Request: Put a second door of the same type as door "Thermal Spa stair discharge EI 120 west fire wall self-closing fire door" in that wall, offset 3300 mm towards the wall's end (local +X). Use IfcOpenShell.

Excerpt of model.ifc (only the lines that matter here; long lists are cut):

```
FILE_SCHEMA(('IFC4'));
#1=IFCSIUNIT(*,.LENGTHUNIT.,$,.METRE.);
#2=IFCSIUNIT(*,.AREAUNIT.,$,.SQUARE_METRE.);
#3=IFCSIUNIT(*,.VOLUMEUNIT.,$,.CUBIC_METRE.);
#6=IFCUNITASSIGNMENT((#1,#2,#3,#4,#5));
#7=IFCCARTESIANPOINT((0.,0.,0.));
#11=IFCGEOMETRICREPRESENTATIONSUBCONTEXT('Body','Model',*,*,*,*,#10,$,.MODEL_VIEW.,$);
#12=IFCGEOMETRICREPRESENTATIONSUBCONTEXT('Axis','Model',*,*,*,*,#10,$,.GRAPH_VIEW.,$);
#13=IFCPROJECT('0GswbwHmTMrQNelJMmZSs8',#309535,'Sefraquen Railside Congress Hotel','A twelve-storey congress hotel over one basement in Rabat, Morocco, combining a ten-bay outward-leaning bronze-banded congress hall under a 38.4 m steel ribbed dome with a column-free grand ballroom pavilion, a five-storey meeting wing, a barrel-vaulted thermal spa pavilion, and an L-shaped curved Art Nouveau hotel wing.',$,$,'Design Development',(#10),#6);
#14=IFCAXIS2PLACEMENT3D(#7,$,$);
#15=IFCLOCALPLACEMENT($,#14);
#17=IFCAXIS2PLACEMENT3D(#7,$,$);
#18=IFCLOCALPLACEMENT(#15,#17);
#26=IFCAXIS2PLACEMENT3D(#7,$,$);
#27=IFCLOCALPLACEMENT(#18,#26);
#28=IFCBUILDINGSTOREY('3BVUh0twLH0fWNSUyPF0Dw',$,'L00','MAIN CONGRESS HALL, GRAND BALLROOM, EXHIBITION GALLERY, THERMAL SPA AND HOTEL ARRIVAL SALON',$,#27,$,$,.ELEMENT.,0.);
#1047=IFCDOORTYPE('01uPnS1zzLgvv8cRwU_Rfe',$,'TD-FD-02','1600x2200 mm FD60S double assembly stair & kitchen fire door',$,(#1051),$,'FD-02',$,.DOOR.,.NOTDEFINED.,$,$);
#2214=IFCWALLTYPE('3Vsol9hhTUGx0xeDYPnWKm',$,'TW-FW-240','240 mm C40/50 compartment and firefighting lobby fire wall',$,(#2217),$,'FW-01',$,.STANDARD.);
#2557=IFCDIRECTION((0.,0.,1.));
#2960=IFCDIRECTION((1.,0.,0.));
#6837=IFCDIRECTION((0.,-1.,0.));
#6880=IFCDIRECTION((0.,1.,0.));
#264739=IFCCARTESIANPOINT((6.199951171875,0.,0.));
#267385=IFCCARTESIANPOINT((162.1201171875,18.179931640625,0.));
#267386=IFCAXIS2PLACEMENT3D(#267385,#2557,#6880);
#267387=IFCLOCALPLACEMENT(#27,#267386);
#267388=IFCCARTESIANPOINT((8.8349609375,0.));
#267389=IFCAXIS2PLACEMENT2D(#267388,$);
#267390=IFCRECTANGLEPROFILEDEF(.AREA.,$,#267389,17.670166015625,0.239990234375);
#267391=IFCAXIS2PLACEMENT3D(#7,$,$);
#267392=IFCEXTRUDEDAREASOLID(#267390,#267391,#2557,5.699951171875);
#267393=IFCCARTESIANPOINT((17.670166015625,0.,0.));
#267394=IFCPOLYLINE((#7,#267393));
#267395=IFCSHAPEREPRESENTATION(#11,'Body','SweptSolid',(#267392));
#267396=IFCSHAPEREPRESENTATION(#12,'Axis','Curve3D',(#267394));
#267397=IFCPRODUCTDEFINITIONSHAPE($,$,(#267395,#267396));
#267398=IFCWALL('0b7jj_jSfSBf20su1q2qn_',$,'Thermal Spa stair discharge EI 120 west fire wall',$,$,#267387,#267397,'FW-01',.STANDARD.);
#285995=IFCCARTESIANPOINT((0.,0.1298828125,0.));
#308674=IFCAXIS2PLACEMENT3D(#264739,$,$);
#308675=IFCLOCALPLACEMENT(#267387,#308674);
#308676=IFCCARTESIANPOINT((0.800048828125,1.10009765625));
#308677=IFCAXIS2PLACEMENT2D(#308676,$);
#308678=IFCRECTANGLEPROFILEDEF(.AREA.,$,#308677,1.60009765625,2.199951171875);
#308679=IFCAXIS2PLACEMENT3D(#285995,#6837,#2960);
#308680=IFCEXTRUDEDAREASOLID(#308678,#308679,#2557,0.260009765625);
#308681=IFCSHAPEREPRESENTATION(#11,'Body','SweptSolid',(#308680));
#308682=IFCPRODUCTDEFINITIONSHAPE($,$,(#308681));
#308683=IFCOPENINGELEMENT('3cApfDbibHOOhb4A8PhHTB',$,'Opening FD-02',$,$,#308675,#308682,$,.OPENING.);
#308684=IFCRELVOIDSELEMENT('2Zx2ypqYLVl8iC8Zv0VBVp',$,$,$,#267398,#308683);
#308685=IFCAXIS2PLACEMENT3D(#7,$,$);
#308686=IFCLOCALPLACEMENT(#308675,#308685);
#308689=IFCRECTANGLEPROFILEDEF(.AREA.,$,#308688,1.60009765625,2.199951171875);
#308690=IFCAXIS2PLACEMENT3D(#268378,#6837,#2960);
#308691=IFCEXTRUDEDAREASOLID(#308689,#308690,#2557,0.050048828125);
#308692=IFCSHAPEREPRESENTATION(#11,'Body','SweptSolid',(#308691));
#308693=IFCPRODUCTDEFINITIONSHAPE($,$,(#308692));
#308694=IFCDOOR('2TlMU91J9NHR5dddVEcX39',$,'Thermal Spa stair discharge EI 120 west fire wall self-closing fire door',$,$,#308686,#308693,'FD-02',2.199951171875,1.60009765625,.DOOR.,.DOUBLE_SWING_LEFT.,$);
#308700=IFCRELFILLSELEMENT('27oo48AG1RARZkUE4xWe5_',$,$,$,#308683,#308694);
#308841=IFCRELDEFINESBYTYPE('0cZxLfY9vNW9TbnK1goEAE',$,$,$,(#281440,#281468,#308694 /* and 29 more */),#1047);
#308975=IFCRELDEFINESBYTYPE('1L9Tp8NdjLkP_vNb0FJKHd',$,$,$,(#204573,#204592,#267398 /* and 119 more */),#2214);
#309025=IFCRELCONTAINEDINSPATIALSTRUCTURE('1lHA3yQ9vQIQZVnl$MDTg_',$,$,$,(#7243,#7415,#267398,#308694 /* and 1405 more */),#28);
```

```python
import ifcopenshell
import ifcopenshell.api.feature
import ifcopenshell.api.geometry
import ifcopenshell.api.root
import ifcopenshell.geom
import ifcopenshell.util.element
import ifcopenshell.util.placement
import ifcopenshell.util.shape
import ifcopenshell.util.unit

model = ifcopenshell.open("model.ifc")
unit_scale = ifcopenshell.util.unit.calculate_unit_scale(model)
settings = ifcopenshell.geom.settings()


def volume(element):
    """Net volume in cubic metres, openings subtracted."""
    shape = ifcopenshell.geom.create_shape(settings, element)
    return ifcopenshell.util.shape.get_volume(shape.geometry)


door = model.by_guid("2TlMU91J9NHR5dddVEcX39")
opening = door.FillsVoids[0].RelatingOpeningElement
wall = opening.VoidsElements[0].RelatingBuildingElement
before = volume(wall)
shift = ifcopenshell.util.placement.get_local_placement(wall.ObjectPlacement)[:3, 0] * 3.3 / unit_scale

# copy_class copies the void relationship, type, container and properties, but no geometry.
new_opening = ifcopenshell.api.root.copy_class(model, product=opening)
new_opening.Representation = ifcopenshell.util.element.copy_deep(
    model, opening.Representation, exclude=["IfcGeometricRepresentationContext", "IfcRepresentationMap"]
)
new_door = ifcopenshell.api.root.copy_class(model, product=door)
new_door.Representation = ifcopenshell.util.element.copy_deep(
    model, door.Representation, exclude=["IfcGeometricRepresentationContext", "IfcRepresentationMap"]
)
new_door.Tag = None
ifcopenshell.api.feature.add_filling(model, opening=new_opening, element=new_door)

for old, new in ((opening, new_opening), (door, new_door)):
    matrix = ifcopenshell.util.placement.get_local_placement(old.ObjectPlacement)
    matrix[:3, 3] += shift
    ifcopenshell.api.geometry.edit_object_placement(model, product=new, matrix=matrix, is_si=False)

after = volume(wall)

print(f"wall volume {before:.3f} -> {after:.3f} m3")

model.write("model_updated.ifc")
```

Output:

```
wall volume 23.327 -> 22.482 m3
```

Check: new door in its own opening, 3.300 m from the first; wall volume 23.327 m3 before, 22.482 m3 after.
